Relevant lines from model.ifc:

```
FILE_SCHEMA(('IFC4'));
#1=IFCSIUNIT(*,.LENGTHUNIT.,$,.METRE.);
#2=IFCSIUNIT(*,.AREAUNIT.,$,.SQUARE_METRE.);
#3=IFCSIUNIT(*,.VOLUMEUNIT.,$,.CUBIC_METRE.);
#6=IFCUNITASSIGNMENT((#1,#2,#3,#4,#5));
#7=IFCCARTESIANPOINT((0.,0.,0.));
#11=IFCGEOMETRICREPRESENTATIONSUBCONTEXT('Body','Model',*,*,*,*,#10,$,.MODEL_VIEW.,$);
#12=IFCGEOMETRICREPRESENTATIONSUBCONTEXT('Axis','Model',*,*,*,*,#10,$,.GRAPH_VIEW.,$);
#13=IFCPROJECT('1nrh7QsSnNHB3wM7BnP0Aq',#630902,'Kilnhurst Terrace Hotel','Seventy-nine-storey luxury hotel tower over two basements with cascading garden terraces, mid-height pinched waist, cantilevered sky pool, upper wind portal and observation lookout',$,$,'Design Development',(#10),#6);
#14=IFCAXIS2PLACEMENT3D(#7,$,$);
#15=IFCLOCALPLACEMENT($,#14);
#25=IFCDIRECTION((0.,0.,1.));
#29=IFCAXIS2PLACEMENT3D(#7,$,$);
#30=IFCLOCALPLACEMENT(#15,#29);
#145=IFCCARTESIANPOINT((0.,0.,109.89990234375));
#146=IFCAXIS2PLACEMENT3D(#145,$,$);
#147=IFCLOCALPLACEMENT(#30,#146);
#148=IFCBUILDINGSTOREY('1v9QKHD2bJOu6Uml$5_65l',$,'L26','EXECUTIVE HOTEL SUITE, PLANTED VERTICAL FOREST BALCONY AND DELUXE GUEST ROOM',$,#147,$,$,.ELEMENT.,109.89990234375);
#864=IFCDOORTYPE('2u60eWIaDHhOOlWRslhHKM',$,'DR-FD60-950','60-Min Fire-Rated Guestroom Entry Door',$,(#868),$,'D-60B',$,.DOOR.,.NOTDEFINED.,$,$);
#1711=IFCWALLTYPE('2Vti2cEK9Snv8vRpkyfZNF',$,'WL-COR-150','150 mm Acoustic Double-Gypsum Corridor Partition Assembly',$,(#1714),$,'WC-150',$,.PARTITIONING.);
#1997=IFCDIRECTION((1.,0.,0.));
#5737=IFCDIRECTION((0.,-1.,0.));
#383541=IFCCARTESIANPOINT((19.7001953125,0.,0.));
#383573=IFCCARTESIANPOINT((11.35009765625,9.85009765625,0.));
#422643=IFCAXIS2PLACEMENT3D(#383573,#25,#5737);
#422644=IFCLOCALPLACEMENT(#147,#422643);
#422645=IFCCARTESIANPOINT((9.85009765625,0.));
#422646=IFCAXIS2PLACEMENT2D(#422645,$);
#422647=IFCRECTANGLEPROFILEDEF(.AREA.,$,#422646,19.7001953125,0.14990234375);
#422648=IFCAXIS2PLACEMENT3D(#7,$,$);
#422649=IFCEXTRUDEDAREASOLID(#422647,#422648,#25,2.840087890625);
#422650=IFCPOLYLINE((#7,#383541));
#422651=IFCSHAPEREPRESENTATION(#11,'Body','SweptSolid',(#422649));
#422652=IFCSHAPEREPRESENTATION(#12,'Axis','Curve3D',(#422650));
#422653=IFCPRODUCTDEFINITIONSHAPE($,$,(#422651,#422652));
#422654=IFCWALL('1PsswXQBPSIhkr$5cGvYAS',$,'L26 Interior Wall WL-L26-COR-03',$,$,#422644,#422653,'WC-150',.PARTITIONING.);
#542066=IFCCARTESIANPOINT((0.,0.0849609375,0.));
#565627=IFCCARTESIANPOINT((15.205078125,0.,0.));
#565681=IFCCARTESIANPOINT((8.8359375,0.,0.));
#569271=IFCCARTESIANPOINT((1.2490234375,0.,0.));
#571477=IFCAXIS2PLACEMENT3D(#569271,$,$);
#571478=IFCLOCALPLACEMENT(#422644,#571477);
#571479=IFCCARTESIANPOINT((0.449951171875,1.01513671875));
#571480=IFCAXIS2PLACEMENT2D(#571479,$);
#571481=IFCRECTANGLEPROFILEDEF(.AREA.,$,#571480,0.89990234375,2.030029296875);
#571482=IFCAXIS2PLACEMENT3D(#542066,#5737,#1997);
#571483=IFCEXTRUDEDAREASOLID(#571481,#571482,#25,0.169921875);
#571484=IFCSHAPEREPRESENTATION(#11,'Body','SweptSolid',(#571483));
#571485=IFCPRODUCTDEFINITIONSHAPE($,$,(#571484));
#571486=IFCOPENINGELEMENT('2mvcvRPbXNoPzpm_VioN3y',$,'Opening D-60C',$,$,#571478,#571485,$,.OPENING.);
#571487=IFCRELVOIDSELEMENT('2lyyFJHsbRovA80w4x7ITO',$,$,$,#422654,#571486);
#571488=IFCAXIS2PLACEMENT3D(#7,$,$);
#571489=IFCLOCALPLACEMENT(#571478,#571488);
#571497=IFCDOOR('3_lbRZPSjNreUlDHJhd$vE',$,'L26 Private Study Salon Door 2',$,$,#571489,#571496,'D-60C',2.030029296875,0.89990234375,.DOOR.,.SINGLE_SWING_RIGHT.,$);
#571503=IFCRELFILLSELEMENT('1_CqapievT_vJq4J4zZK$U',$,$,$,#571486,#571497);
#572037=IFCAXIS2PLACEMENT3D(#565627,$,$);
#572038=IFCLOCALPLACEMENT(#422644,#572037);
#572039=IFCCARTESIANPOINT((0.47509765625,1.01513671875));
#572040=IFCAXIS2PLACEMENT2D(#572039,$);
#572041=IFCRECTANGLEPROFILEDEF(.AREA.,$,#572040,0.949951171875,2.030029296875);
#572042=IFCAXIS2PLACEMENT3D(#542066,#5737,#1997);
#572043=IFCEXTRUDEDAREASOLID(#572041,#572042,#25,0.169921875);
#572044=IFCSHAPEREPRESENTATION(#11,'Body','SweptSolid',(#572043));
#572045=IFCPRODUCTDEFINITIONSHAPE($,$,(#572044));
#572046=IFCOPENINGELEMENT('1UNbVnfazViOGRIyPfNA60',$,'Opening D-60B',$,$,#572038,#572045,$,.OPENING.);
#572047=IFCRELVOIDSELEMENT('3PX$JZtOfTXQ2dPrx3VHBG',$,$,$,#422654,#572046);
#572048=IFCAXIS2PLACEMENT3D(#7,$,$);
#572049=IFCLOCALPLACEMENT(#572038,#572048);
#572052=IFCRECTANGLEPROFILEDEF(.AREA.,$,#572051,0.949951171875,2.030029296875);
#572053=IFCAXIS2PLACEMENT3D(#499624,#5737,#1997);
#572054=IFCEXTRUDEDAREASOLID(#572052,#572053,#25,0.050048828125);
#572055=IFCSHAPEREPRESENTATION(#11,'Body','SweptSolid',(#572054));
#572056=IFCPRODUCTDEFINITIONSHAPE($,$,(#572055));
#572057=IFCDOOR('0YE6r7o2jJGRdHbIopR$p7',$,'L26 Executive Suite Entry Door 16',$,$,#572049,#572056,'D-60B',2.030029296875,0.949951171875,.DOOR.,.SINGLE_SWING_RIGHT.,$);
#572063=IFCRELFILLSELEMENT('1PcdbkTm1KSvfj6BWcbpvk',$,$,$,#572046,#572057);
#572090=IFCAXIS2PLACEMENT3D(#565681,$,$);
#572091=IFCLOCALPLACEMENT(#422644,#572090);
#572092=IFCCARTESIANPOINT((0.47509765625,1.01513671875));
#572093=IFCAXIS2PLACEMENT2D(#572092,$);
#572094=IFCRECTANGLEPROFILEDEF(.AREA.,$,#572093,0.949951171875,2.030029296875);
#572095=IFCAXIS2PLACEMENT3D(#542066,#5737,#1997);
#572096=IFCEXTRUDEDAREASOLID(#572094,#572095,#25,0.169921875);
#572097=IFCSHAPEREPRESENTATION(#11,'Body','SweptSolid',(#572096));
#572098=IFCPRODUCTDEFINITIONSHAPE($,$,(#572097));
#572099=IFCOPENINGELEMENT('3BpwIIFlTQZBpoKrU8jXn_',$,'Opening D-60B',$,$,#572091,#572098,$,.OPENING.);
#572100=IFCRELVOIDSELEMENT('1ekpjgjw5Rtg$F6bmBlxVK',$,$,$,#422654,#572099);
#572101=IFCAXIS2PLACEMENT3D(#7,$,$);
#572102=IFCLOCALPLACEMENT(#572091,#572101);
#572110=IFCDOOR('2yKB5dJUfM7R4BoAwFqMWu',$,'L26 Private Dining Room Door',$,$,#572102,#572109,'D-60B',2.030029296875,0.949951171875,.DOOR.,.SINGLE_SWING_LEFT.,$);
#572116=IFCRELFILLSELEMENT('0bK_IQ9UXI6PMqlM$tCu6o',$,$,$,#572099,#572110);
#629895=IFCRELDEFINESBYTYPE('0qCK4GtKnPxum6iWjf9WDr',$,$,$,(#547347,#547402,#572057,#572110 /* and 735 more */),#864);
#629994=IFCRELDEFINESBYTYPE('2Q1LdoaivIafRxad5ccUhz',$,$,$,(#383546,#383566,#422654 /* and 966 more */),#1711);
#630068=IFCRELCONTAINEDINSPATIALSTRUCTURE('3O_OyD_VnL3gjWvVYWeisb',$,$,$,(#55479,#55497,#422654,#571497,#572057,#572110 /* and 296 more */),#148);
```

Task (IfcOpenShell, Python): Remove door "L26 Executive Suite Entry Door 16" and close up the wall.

```python
import ifcopenshell
import ifcopenshell.api.feature
import ifcopenshell.api.root
import ifcopenshell.geom
import ifcopenshell.util.shape

model = ifcopenshell.open("model.ifc")
settings = ifcopenshell.geom.settings()


def volume(element):
    """Net volume in cubic metres, openings subtracted."""
    shape = ifcopenshell.geom.create_shape(settings, element)
    return ifcopenshell.util.shape.get_volume(shape.geometry)


door = model.by_guid("0YE6r7o2jJGRdHbIopR$p7")
opening = door.FillsVoids[0].RelatingOpeningElement
wall = opening.VoidsElements[0].RelatingBuildingElement
before = volume(wall)

ifcopenshell.api.root.remove_product(model, product=door)
ifcopenshell.api.feature.remove_feature(model, feature=opening)

after = volume(wall)

print(f"wall volume {before:.3f} -> {after:.3f} m3")

model.write("model_edited.ifc")
```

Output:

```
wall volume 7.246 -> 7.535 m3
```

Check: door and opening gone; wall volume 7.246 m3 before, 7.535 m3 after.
